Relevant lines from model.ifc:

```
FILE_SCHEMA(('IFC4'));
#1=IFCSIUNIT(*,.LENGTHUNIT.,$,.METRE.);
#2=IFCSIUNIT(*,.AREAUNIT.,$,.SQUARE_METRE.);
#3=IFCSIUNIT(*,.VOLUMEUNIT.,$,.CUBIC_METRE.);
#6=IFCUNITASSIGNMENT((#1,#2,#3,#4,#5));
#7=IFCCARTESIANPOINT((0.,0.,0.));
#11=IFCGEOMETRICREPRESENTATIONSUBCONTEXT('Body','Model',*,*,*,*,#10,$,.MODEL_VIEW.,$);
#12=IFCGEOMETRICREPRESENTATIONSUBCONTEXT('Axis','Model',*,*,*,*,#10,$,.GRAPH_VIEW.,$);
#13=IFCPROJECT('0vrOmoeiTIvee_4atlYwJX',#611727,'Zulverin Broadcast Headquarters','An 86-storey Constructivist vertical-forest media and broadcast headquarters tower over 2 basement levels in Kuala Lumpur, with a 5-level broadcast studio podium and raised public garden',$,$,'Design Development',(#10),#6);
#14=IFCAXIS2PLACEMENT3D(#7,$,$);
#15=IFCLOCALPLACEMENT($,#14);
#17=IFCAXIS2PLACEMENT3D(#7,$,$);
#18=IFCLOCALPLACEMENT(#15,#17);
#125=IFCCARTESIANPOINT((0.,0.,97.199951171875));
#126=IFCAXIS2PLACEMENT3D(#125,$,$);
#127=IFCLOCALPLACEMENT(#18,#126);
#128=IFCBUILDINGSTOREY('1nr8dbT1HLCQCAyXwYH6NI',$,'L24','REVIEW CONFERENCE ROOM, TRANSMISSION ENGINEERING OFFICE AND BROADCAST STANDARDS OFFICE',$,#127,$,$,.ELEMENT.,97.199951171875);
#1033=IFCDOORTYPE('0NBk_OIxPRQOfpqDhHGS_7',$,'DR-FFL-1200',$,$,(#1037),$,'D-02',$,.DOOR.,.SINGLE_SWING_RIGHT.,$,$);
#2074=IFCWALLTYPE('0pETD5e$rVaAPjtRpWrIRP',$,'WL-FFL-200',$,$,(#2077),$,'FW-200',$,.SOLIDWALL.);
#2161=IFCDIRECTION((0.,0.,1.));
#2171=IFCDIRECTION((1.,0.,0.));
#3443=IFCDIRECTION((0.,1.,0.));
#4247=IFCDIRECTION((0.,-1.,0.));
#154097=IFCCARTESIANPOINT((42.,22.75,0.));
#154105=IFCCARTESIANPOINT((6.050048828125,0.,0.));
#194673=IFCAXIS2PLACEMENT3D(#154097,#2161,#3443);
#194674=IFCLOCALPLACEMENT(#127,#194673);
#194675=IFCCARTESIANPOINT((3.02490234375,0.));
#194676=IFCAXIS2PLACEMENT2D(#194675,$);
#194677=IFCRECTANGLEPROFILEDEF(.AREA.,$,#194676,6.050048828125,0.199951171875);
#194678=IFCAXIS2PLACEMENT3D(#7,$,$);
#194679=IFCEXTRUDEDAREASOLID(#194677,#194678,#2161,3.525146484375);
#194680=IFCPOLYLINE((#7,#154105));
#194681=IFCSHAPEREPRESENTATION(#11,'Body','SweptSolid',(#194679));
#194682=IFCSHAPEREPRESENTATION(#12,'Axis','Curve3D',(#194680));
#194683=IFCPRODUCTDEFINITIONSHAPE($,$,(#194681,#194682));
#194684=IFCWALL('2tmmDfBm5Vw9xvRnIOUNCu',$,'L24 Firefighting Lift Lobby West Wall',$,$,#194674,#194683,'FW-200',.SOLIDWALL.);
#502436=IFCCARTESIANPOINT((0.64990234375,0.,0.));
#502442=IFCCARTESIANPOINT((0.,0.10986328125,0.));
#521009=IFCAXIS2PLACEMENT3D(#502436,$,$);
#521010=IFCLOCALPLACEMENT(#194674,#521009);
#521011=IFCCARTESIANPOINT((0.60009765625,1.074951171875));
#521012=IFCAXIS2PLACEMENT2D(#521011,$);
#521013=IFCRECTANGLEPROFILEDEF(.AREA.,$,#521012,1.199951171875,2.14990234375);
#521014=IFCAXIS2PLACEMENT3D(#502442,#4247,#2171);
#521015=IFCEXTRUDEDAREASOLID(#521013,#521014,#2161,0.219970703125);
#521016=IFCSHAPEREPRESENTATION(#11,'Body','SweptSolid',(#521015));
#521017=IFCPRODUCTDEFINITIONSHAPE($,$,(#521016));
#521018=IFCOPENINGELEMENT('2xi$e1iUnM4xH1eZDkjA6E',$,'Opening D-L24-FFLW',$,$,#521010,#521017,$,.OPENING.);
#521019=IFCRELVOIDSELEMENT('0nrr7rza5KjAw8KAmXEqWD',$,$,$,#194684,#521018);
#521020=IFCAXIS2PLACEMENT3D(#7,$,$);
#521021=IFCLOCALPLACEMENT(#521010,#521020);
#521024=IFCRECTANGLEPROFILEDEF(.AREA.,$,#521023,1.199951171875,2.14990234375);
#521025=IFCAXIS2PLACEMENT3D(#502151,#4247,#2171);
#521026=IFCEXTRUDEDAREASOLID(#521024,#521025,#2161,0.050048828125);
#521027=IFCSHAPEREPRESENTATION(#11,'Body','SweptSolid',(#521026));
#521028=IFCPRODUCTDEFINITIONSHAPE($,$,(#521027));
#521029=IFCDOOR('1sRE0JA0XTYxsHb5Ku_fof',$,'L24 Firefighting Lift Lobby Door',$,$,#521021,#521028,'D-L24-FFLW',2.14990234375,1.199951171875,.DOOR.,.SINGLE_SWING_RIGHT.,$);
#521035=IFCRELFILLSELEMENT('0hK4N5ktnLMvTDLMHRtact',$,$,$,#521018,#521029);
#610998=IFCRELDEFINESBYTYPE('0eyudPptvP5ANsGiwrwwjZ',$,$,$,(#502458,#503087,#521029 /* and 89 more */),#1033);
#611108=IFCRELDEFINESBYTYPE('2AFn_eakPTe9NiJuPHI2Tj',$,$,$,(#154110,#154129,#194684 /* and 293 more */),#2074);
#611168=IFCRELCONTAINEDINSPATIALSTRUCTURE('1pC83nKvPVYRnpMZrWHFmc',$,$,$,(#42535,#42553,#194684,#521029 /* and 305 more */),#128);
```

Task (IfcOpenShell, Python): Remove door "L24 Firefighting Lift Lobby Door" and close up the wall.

```python
import ifcopenshell
import ifcopenshell.api.feature
import ifcopenshell.api.root
import ifcopenshell.geom
import ifcopenshell.util.shape

model = ifcopenshell.open("model.ifc")
settings = ifcopenshell.geom.settings()


def volume(element):
    """Net volume in cubic metres, openings subtracted."""
    shape = ifcopenshell.geom.create_shape(settings, element)
    return ifcopenshell.util.shape.get_volume(shape.geometry)


door = model.by_guid("1sRE0JA0XTYxsHb5Ku_fof")
opening = door.FillsVoids[0].RelatingOpeningElement
wall = opening.VoidsElements[0].RelatingBuildingElement
before = volume(wall)

ifcopenshell.api.root.remove_product(model, product=door)
ifcopenshell.api.feature.remove_feature(model, feature=opening)

after = volume(wall)

print(f"wall volume {before:.3f} -> {after:.3f} m3")

model.write("model-out.ifc")
```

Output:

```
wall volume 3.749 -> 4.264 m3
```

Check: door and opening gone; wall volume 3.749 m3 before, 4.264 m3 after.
